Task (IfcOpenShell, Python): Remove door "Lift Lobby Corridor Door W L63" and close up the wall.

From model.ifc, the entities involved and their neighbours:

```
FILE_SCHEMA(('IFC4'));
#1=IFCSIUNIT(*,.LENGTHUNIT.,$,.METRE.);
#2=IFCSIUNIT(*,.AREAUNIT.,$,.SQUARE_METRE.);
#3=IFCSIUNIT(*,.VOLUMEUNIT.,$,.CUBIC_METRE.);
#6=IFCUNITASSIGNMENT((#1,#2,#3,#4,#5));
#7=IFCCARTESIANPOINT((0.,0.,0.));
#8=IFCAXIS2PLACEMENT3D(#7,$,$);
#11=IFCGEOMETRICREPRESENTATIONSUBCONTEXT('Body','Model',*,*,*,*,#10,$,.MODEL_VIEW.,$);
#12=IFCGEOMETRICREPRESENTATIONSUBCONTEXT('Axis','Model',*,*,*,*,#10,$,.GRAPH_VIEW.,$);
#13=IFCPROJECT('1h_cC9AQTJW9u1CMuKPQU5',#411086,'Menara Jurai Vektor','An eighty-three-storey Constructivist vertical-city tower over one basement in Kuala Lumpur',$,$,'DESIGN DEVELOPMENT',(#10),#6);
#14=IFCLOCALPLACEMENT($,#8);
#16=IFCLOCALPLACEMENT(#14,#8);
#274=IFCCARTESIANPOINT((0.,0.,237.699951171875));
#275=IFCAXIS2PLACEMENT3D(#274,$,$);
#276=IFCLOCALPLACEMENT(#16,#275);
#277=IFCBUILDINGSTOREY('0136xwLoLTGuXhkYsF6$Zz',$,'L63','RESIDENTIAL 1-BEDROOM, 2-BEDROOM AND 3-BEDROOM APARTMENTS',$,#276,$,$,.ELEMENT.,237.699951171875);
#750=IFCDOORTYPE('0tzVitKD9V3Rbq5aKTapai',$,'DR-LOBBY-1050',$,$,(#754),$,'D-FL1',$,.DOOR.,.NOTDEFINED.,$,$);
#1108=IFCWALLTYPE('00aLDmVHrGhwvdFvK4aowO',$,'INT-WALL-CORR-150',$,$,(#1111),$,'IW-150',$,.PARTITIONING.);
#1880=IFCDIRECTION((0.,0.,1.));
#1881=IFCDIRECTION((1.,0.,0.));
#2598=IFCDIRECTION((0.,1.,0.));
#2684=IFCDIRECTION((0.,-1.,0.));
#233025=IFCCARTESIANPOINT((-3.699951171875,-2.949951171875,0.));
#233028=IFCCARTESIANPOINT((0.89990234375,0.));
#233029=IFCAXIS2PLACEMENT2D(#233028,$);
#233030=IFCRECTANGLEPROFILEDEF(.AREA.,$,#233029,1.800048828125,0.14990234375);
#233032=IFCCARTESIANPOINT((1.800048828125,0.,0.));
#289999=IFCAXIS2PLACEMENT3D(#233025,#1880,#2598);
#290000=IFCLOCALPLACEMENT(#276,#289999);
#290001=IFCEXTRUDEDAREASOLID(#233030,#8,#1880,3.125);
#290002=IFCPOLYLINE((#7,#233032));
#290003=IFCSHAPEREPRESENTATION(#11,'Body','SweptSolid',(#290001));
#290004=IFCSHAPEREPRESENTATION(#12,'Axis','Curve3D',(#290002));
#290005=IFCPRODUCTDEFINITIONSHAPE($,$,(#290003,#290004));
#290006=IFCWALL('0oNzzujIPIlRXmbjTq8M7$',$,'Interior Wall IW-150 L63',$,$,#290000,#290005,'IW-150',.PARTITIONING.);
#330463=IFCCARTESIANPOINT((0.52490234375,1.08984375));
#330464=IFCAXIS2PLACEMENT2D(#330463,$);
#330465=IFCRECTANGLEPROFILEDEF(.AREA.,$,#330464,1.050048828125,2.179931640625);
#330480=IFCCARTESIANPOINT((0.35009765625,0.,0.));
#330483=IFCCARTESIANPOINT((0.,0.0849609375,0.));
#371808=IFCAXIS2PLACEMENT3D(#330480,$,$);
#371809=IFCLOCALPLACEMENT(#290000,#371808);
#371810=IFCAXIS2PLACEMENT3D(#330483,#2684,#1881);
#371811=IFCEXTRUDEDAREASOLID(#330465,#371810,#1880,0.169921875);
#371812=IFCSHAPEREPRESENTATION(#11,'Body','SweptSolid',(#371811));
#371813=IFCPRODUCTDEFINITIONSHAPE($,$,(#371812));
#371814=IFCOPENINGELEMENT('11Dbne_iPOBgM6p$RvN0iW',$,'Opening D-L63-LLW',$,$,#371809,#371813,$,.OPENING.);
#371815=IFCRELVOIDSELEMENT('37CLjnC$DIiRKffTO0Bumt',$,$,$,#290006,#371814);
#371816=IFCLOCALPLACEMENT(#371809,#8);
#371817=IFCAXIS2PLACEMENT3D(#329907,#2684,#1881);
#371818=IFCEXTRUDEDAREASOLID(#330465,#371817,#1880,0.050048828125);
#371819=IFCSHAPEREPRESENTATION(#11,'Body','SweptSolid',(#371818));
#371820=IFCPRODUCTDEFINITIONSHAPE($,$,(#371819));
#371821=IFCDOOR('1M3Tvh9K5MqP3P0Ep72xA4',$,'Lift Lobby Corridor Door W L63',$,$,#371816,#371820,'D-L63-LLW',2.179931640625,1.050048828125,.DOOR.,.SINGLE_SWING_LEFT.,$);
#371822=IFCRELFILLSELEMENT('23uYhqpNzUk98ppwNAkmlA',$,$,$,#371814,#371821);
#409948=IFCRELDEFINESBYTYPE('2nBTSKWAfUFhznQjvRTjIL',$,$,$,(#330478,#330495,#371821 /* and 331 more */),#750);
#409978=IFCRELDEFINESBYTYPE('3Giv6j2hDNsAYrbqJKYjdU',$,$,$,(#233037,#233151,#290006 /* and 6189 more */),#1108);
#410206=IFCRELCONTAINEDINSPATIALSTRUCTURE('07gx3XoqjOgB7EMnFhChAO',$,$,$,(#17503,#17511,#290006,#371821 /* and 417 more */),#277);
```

```python
import ifcopenshell
import ifcopenshell.api.feature
import ifcopenshell.api.root
import ifcopenshell.geom
import ifcopenshell.util.shape

model = ifcopenshell.open("model.ifc")
settings = ifcopenshell.geom.settings()


def volume(element):
    """Net volume in cubic metres, openings subtracted."""
    shape = ifcopenshell.geom.create_shape(settings, element)
    return ifcopenshell.util.shape.get_volume(shape.geometry)


door = model.by_id(371821)
opening = door.FillsVoids[0].RelatingOpeningElement
wall = opening.VoidsElements[0].RelatingBuildingElement
before = volume(wall)

ifcopenshell.api.root.remove_product(model, product=door)
ifcopenshell.api.feature.remove_feature(model, feature=opening)

after = volume(wall)

print(f"wall volume {before:.3f} -> {after:.3f} m3")

model.write("model_edited.ifc")
```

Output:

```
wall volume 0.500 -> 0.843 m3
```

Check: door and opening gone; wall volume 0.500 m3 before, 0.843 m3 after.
